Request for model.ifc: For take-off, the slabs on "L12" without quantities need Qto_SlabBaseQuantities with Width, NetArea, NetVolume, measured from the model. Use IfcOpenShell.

First a look at what the model holds.

```python
import ifcopenshell
import ifcopenshell.util.element
import ifcopenshell.util.unit

model = ifcopenshell.open("model.ifc")
print(model.schema)
for unit_type in ("LENGTHUNIT", "AREAUNIT", "VOLUMEUNIT"):
    print(unit_type, ifcopenshell.util.unit.calculate_unit_scale(model, unit_type))
storey = next(s for s in model.by_type("IfcBuildingStorey") if s.Name == "L12")
slabs = [e for e in ifcopenshell.util.element.get_decomposition(storey) if e.is_a("IfcSlab")]
for e in sorted(slabs, key=lambda e: e.id()):
    print(e.id(), e.is_a(), e.Name, list(ifcopenshell.util.element.get_psets(e, qtos_only=True)), sep=" | ")
```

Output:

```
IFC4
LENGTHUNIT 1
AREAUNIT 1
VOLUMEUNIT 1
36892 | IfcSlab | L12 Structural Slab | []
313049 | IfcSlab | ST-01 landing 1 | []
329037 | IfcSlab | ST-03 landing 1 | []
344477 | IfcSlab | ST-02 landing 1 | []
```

```python
import ifcopenshell
import ifcopenshell.api.pset
import ifcopenshell.geom
import ifcopenshell.util.element
import ifcopenshell.util.shape
import ifcopenshell.util.unit

model = ifcopenshell.open("model.ifc")
unit_scale = ifcopenshell.util.unit.calculate_unit_scale(model)
area_scale = ifcopenshell.util.unit.calculate_unit_scale(model, "AREAUNIT")
volume_scale = ifcopenshell.util.unit.calculate_unit_scale(model, "VOLUMEUNIT")
settings = ifcopenshell.geom.settings()

storey = next(s for s in model.by_type("IfcBuildingStorey") if s.Name == "L12")
slabs = [e for e in ifcopenshell.util.element.get_decomposition(storey) if e.is_a("IfcSlab")]

for e in sorted(slabs, key=lambda e: e.id()):
    if ifcopenshell.util.element.get_psets(e, qtos_only=True, should_inherit=False):
        continue
    # Geometry comes back in metres, in the element's own axes.
    shape = ifcopenshell.geom.create_shape(settings, e)
    values = {
        "Width": ifcopenshell.util.shape.get_z(shape.geometry) / unit_scale,
        "NetArea": ifcopenshell.util.shape.get_footprint_area(shape.geometry) / area_scale,
        "NetVolume": ifcopenshell.util.shape.get_volume(shape.geometry) / volume_scale,
    }
    qto = ifcopenshell.api.pset.add_qto(model, product=e, name="Qto_SlabBaseQuantities")
    ifcopenshell.api.pset.edit_qto(model, qto=qto, properties=values)
    print(e.id(), {k: round(v, 3) for k, v in values.items()})

model.write("model-out.ifc")
```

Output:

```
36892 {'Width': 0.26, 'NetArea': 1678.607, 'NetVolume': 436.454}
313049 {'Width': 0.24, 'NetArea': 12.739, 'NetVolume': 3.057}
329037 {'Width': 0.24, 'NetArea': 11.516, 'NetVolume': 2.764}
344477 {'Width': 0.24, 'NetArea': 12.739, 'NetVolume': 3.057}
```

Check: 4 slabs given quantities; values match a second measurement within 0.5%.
